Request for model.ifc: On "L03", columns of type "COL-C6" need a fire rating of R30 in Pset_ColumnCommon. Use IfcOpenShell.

First a look at what the model holds.

```python
import ifcopenshell
import ifcopenshell.util.element

model = ifcopenshell.open("model.ifc")
print(model.schema)
storey = next(s for s in model.by_type("IfcBuildingStorey") if s.Name == "L03")
columns = [e for e in ifcopenshell.util.element.get_decomposition(storey) if e.is_a("IfcColumn")]
seen = {}
for e in columns:
    element_type = ifcopenshell.util.element.get_type(e)
    key = (element_type.Name if element_type != e and element_type else None, ifcopenshell.util.element.get_pset(e, "Pset_ColumnCommon", "FireRating"))
    seen[key] = seen.get(key, 0) + 1
for (name, value), count in sorted(seen.items(), key=str):
    print(count, "x", name, "|", value)
```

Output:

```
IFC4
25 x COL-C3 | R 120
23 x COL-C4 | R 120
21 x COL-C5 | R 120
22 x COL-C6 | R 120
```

```python
import ifcopenshell
import ifcopenshell.api.pset
import ifcopenshell.util.element

model = ifcopenshell.open("model.ifc")

storey = next(s for s in model.by_type("IfcBuildingStorey") if s.Name == "L03")
columns = [e for e in ifcopenshell.util.element.get_decomposition(storey) if e.is_a("IfcColumn")]

count = 0
for e in columns:
    element_type = ifcopenshell.util.element.get_type(e)
    if element_type in (None, e) or element_type.Name != "COL-C6":
        continue
    # add_pset returns the element's existing set when there is one.
    pset = ifcopenshell.api.pset.add_pset(model, product=e, name="Pset_ColumnCommon")
    ifcopenshell.api.pset.edit_pset(model, pset=pset, properties={"FireRating": "R30"})
    count += 1

print(count, "columns updated")

model.write("model_updated.ifc")
```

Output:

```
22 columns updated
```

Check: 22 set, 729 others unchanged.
